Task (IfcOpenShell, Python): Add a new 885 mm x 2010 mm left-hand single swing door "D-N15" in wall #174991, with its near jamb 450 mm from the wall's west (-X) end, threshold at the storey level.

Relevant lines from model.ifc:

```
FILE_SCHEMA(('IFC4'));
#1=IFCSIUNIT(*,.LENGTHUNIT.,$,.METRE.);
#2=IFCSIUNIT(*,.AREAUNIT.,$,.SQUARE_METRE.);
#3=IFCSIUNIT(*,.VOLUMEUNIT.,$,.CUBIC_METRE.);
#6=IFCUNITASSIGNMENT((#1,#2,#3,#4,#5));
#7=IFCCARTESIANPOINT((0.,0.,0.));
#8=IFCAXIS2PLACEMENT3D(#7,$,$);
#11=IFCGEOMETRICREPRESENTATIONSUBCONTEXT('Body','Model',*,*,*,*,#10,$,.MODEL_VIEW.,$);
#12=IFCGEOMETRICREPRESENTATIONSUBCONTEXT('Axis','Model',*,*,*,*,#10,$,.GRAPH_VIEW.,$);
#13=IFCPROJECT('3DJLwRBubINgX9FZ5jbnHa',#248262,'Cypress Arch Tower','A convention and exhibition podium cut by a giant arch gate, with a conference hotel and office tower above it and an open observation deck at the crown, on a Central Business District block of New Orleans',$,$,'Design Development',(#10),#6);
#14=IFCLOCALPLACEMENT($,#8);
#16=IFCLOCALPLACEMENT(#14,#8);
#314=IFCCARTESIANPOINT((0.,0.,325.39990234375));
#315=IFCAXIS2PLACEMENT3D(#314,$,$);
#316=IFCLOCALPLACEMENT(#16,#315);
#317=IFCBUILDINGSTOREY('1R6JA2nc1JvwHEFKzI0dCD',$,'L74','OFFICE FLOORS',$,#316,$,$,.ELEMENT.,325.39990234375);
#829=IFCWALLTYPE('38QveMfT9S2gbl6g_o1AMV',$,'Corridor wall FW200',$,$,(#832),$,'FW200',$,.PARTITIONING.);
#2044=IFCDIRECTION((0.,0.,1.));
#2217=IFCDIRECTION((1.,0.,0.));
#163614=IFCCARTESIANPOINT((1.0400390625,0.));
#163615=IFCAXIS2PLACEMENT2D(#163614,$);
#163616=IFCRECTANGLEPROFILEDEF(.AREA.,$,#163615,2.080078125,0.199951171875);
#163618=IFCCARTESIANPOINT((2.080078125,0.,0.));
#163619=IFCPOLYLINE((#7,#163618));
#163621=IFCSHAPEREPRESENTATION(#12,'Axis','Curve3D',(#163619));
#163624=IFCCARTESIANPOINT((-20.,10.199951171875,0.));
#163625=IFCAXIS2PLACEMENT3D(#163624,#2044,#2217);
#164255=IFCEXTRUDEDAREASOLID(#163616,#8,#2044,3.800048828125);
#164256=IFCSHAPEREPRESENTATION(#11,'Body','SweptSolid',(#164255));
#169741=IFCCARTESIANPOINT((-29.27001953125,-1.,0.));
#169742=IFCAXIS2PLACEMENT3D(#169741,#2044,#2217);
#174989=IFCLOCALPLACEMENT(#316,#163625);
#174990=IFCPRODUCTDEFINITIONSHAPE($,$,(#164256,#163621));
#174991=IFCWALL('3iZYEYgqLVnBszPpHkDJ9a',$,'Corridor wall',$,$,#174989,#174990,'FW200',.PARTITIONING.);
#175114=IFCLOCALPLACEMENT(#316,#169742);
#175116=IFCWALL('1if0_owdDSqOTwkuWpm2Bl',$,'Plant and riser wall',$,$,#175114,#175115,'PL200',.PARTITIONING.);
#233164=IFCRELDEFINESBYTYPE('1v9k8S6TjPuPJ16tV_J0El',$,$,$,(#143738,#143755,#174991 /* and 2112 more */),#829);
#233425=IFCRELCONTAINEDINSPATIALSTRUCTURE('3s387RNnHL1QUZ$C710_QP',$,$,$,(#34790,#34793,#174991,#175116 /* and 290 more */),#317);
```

```python
import numpy as np
import ifcopenshell
import ifcopenshell.api.feature
import ifcopenshell.api.geometry
import ifcopenshell.api.root
import ifcopenshell.api.spatial
import ifcopenshell.geom
import ifcopenshell.util.element
import ifcopenshell.util.placement
import ifcopenshell.util.representation
import ifcopenshell.util.shape
import ifcopenshell.util.unit

model = ifcopenshell.open("model.ifc")
unit_scale = ifcopenshell.util.unit.calculate_unit_scale(model)
settings = ifcopenshell.geom.settings()


def volume(element):
    """Net volume in cubic metres, openings subtracted."""
    shape = ifcopenshell.geom.create_shape(settings, element)
    return ifcopenshell.util.shape.get_volume(shape.geometry)


wall = model.by_id(174991)
storey = ifcopenshell.util.element.get_container(wall, ifc_class="IfcBuildingStorey")
context = ifcopenshell.util.representation.get_context(model, "Model", "Body", "MODEL_VIEW")
before = volume(wall)

width, height, from_end, sill = 0.885, 2.01, 0.45, 0.0  # metres

# The wall runs along its own X axis, and the end named is its -X end.
wall_shape = ifcopenshell.geom.create_shape(settings, wall)
x, y, z = ifcopenshell.util.shape.get_vertices(wall_shape.geometry).T
start = x.min() + from_end
face, thickness = float(y.min()), float(y.max() - y.min())
wall_matrix = ifcopenshell.util.placement.get_local_placement(wall.ObjectPlacement)
level = ifcopenshell.util.placement.get_local_placement(storey.ObjectPlacement)[2, 3]


def in_wall(x, y):
    """Placement at x, y metres in the wall's axes, at sill height."""
    matrix = wall_matrix.copy()
    matrix[:, 3] = wall_matrix @ np.array([x / unit_scale, y / unit_scale, 0.0, 1.0])
    matrix[2, 3] = level + sill / unit_scale
    return matrix


# Opening: a box that overshoots both wall faces by 50 mm.
opening = ifcopenshell.api.root.create_entity(model, ifc_class="IfcOpeningElement", predefined_type="OPENING")
box = ifcopenshell.api.geometry.add_wall_representation(
    model, context=context, length=width, height=height, thickness=thickness + 0.1
)
ifcopenshell.api.geometry.assign_representation(model, product=opening, representation=box)
ifcopenshell.api.geometry.edit_object_placement(model, product=opening, matrix=in_wall(start, face - 0.05), is_si=False)
ifcopenshell.api.feature.add_feature(model, feature=opening, element=wall)

door = ifcopenshell.api.root.create_entity(model, ifc_class="IfcDoor", name="D-N15", predefined_type="DOOR")
door.OverallWidth, door.OverallHeight = width / unit_scale, height / unit_scale
door.OperationType = "SINGLE_SWING_LEFT"
body = ifcopenshell.api.geometry.add_door_representation(
    model,
    context=context,
    overall_width=door.OverallWidth,
    overall_height=door.OverallHeight,
    operation_type="SINGLE_SWING_LEFT",
    lining_properties={"LiningDepth": thickness / unit_scale, "ThresholdDepth": thickness / unit_scale},
)
ifcopenshell.api.geometry.assign_representation(model, product=door, representation=body)
ifcopenshell.api.spatial.assign_container(model, products=[door], relating_structure=storey)
ifcopenshell.api.feature.add_filling(model, opening=opening, element=door)

# The lining spans the wall, so the door starts at the wall face.
ifcopenshell.api.geometry.edit_object_placement(model, product=door, matrix=in_wall(start, face), is_si=False)

after = volume(wall)

print(f"wall volume {before:.3f} -> {after:.3f} m3")

model.write("model_v2.ifc")
```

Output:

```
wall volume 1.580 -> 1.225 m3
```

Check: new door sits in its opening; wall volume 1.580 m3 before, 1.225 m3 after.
